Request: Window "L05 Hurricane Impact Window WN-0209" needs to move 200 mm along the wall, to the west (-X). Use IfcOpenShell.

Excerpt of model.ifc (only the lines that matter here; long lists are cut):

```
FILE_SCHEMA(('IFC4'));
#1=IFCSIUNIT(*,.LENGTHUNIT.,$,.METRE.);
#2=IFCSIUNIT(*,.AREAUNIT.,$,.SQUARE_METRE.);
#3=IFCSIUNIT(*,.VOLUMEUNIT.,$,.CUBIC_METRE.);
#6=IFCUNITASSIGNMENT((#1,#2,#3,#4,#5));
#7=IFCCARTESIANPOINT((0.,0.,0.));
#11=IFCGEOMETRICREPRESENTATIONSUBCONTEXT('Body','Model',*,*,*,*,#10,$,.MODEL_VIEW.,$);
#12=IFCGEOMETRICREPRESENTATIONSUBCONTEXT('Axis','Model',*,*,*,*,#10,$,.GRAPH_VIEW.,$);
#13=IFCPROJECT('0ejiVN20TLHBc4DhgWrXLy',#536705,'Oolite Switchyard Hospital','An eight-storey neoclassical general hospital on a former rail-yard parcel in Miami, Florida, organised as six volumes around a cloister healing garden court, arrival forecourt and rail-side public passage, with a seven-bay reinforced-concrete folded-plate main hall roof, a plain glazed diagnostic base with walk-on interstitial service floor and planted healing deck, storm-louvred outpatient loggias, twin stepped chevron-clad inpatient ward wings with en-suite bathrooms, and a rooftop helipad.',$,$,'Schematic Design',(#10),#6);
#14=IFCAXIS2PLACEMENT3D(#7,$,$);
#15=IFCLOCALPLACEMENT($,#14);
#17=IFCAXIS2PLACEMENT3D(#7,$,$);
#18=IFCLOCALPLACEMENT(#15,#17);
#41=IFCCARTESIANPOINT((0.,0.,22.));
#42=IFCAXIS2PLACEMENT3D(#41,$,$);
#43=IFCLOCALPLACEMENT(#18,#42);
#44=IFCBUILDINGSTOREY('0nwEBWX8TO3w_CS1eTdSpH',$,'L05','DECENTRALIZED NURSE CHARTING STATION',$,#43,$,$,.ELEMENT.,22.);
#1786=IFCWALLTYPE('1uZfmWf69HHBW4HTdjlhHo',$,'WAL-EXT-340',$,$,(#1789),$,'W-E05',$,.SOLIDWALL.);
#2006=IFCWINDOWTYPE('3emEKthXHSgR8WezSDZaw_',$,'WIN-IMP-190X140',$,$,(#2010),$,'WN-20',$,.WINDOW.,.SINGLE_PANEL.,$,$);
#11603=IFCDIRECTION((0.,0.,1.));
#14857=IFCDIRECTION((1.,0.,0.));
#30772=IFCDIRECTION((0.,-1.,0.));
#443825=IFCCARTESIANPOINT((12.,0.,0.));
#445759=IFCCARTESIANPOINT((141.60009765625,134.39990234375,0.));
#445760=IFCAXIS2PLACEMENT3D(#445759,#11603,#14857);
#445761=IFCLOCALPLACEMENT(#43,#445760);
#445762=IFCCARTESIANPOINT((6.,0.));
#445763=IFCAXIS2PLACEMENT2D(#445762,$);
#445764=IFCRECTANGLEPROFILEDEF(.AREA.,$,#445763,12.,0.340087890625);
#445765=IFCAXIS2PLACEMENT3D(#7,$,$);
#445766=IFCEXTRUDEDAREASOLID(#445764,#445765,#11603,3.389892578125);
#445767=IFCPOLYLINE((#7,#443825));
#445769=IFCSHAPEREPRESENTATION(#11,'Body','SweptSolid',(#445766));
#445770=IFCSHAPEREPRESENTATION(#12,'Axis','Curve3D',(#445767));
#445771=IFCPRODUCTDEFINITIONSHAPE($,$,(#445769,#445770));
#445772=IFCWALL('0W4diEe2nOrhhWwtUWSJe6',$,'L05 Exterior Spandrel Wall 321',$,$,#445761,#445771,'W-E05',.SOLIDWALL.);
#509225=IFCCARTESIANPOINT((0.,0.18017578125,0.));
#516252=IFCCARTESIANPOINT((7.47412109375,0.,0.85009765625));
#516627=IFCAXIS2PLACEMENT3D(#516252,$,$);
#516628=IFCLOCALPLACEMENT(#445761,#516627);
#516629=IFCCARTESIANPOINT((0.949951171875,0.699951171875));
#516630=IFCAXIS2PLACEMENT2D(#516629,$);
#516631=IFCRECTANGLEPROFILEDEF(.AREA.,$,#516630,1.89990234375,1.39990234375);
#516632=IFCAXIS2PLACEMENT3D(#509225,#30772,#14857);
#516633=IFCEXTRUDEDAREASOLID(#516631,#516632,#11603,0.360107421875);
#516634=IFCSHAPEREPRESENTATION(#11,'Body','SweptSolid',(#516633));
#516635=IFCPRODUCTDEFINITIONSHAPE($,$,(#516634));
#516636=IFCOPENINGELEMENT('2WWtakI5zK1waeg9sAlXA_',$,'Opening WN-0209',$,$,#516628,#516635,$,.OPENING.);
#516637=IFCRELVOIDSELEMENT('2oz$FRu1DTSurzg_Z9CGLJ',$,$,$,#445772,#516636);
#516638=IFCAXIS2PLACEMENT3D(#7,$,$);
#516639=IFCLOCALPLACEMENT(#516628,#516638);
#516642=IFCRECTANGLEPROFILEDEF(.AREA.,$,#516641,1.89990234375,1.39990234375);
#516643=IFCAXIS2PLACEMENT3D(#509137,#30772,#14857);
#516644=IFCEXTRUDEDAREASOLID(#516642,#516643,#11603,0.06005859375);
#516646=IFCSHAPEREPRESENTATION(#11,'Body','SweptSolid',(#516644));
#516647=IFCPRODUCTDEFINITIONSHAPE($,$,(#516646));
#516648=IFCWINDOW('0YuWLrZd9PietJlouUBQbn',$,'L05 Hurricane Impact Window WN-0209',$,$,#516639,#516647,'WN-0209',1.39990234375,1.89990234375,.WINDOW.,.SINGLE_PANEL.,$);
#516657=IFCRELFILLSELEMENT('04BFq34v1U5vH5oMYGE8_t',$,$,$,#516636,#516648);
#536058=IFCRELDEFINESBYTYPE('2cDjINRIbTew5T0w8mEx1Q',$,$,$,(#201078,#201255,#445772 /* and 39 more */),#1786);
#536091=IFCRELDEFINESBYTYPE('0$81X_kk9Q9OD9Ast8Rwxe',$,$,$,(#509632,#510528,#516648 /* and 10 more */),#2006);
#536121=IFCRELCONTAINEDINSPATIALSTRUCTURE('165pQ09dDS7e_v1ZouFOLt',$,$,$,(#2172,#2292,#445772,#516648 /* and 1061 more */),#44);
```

```python
import ifcopenshell
import ifcopenshell.api.geometry
import ifcopenshell.util.placement
import ifcopenshell.util.unit

model = ifcopenshell.open("model.ifc")
unit_scale = ifcopenshell.util.unit.calculate_unit_scale(model)

window = model.by_guid("0YuWLrZd9PietJlouUBQbn")
opening = window.FillsVoids[0].RelatingOpeningElement
wall = opening.VoidsElements[0].RelatingBuildingElement

wall_matrix = ifcopenshell.util.placement.get_local_placement(wall.ObjectPlacement)
shift = wall_matrix[:3, 0] * -0.2 / unit_scale
before = ifcopenshell.util.placement.get_local_placement(window.ObjectPlacement)[:3, 3].copy()

# The window is placed relative to its opening, so it follows when the opening moves.
matrix = ifcopenshell.util.placement.get_local_placement(opening.ObjectPlacement)
matrix[:3, 3] += shift
ifcopenshell.api.geometry.edit_object_placement(
    model, product=opening, matrix=matrix, is_si=False, should_transform_children=True
)

after = ifcopenshell.util.placement.get_local_placement(window.ObjectPlacement)[:3, 3]
print("window moved by", (after - before).round(3) + 0.0)

model.write("model_v2.ifc")
```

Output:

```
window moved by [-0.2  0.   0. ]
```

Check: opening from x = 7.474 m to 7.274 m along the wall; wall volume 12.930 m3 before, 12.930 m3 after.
